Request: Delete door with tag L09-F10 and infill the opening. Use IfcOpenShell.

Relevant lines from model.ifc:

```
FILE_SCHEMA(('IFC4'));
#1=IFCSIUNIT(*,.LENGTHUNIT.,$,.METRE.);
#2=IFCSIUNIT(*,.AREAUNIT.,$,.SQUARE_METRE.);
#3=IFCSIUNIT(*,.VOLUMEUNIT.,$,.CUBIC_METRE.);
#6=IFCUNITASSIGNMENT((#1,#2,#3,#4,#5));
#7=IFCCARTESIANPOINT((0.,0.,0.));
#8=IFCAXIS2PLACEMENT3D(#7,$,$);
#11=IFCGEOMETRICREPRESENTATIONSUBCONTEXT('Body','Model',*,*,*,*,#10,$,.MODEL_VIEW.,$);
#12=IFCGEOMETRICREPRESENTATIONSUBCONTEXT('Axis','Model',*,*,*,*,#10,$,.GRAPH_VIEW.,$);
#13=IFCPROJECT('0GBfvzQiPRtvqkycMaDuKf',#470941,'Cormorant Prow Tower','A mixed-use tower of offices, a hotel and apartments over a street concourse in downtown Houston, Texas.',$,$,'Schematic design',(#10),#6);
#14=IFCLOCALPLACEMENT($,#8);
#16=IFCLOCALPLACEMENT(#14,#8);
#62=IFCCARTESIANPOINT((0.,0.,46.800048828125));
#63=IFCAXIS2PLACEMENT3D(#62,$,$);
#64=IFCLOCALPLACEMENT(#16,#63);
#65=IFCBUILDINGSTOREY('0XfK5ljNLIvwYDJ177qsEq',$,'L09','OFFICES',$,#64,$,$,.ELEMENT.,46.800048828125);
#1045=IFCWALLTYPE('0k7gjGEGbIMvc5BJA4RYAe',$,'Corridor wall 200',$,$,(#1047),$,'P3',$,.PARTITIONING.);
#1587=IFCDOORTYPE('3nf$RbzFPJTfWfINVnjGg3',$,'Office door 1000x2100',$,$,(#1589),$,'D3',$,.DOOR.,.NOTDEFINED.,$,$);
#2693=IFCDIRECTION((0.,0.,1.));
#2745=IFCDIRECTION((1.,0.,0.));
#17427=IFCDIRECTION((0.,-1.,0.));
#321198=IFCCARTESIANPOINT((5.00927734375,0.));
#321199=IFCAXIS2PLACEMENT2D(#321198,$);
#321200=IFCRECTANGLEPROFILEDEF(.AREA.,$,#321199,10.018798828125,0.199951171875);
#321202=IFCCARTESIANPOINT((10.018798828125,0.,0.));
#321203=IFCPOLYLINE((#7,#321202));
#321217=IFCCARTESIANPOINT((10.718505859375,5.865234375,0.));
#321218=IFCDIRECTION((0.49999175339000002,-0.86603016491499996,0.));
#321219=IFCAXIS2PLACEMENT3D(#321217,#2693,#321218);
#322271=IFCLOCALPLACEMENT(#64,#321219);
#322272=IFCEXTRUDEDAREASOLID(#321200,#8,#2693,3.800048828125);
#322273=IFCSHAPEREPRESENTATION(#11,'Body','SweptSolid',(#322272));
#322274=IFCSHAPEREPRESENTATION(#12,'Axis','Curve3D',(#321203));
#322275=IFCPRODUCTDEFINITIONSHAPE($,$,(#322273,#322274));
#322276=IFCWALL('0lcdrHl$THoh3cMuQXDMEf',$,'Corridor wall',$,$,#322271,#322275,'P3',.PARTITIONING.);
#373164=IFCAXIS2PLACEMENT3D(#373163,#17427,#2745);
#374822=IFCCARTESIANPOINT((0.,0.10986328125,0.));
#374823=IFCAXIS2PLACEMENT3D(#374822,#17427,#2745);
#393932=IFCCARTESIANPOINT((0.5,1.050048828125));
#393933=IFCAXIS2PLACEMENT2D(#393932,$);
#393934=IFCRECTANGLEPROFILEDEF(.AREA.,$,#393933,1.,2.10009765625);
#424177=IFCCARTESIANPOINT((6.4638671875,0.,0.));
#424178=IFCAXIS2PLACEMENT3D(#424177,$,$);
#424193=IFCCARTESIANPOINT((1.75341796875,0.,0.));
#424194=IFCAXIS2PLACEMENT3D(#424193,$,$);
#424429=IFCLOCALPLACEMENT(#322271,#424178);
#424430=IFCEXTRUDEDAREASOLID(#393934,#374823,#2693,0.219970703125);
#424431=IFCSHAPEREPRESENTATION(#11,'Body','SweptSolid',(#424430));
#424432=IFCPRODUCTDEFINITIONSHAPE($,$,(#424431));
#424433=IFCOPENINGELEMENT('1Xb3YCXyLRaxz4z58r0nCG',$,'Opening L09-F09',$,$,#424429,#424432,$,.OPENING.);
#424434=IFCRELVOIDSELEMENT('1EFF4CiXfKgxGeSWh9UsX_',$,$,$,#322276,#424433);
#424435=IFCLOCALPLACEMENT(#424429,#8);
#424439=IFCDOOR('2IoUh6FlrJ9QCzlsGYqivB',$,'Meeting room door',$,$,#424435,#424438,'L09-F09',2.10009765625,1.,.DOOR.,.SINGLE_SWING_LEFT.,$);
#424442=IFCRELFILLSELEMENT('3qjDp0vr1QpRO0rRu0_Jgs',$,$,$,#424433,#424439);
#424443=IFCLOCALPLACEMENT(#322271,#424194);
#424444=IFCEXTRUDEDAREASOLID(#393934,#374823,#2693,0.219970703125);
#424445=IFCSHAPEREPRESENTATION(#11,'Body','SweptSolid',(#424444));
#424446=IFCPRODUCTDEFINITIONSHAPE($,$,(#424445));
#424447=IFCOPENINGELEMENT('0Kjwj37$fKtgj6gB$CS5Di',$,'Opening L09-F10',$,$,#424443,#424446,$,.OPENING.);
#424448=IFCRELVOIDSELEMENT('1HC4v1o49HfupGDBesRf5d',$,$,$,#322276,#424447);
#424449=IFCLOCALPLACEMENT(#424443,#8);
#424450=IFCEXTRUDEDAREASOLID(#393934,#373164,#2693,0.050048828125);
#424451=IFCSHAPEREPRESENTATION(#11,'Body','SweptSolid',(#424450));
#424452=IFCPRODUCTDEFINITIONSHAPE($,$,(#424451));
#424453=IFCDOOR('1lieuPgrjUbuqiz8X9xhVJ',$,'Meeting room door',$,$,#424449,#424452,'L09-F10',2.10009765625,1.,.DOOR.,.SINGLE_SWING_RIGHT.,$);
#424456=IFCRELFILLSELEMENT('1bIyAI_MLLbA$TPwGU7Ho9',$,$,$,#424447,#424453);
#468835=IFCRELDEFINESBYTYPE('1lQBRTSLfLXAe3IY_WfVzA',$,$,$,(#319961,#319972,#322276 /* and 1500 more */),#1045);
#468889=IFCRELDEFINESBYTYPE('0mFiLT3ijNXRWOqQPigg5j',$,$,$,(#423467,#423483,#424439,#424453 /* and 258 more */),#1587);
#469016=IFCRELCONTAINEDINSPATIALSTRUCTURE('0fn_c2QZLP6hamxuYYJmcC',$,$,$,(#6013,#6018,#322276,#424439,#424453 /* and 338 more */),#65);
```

```python
import ifcopenshell
import ifcopenshell.api.feature
import ifcopenshell.api.root
import ifcopenshell.geom
import ifcopenshell.util.shape

model = ifcopenshell.open("model.ifc")
settings = ifcopenshell.geom.settings()


def volume(element):
    """Net volume in cubic metres, openings subtracted."""
    shape = ifcopenshell.geom.create_shape(settings, element)
    return ifcopenshell.util.shape.get_volume(shape.geometry)


door = model.by_guid("1lieuPgrjUbuqiz8X9xhVJ")
opening = door.FillsVoids[0].RelatingOpeningElement
wall = opening.VoidsElements[0].RelatingBuildingElement
before = volume(wall)

ifcopenshell.api.root.remove_product(model, product=door)
ifcopenshell.api.feature.remove_feature(model, feature=opening)

after = volume(wall)

print(f"wall volume {before:.3f} -> {after:.3f} m3")

model.write("model_rev.ifc")
```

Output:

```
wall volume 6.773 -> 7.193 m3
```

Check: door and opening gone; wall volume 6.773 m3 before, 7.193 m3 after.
